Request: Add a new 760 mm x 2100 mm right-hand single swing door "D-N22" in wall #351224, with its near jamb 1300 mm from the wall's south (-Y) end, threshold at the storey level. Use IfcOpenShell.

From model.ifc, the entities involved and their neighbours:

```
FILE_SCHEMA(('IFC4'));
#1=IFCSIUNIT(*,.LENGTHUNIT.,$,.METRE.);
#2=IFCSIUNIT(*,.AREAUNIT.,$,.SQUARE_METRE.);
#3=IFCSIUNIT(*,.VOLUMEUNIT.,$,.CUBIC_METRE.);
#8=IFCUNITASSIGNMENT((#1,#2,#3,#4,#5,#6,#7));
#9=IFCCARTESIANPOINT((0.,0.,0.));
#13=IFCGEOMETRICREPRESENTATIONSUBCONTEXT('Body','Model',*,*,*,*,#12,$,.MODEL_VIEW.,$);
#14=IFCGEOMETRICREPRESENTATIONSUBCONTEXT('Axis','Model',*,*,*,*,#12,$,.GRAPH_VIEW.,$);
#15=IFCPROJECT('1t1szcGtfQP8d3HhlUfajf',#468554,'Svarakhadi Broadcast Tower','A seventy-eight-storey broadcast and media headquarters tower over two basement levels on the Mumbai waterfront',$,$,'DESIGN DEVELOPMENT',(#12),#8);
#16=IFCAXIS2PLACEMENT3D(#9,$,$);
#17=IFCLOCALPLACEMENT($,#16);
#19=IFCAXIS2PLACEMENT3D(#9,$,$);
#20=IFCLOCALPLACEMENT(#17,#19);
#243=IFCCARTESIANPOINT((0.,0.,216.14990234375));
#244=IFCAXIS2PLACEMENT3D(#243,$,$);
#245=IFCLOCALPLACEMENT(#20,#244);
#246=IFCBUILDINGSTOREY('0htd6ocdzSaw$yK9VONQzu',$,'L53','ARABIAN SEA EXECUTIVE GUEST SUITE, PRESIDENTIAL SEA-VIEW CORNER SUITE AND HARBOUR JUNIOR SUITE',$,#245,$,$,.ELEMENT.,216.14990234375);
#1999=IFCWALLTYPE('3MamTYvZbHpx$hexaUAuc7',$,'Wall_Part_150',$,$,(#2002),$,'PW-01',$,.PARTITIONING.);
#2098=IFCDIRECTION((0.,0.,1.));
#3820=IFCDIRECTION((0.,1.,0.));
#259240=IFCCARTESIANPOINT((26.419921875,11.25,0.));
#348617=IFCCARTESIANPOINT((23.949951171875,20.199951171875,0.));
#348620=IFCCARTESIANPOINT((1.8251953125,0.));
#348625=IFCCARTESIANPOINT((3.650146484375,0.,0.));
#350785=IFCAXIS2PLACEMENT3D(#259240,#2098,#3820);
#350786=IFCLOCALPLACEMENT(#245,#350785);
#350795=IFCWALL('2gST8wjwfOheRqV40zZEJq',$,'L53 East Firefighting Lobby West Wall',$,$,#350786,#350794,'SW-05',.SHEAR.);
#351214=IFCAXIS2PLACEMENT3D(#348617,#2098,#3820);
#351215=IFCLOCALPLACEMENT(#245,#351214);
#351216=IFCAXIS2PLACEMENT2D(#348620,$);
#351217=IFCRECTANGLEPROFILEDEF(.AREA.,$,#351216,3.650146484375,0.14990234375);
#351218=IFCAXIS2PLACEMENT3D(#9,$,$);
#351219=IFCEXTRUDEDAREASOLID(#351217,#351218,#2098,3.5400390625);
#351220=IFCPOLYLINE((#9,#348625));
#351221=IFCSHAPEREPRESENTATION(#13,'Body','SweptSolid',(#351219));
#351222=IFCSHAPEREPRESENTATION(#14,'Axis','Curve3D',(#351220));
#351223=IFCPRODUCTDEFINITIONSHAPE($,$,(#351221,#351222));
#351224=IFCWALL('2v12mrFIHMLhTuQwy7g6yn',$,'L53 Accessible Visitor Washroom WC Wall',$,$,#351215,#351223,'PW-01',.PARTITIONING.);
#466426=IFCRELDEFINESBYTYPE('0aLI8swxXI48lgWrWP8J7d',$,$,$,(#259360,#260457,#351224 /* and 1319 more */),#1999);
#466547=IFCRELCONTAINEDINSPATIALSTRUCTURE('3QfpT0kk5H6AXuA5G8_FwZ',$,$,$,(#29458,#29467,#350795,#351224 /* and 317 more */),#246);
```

```python
import numpy as np
import ifcopenshell
import ifcopenshell.api.feature
import ifcopenshell.api.geometry
import ifcopenshell.api.root
import ifcopenshell.api.spatial
import ifcopenshell.geom
import ifcopenshell.util.element
import ifcopenshell.util.placement
import ifcopenshell.util.representation
import ifcopenshell.util.shape
import ifcopenshell.util.unit

model = ifcopenshell.open("model.ifc")
unit_scale = ifcopenshell.util.unit.calculate_unit_scale(model)
settings = ifcopenshell.geom.settings()


def volume(element):
    """Net volume in cubic metres, openings subtracted."""
    shape = ifcopenshell.geom.create_shape(settings, element)
    return ifcopenshell.util.shape.get_volume(shape.geometry)


wall = model.by_id(351224)
storey = ifcopenshell.util.element.get_container(wall, ifc_class="IfcBuildingStorey")
context = ifcopenshell.util.representation.get_context(model, "Model", "Body", "MODEL_VIEW")
before = volume(wall)

width, height, from_end, sill = 0.76, 2.1, 1.3, 0.0  # metres

# The wall runs along its own X axis, and the end named is its -X end.
wall_shape = ifcopenshell.geom.create_shape(settings, wall)
x, y, z = ifcopenshell.util.shape.get_vertices(wall_shape.geometry).T
start = x.min() + from_end
face, thickness = float(y.min()), float(y.max() - y.min())
wall_matrix = ifcopenshell.util.placement.get_local_placement(wall.ObjectPlacement)
level = ifcopenshell.util.placement.get_local_placement(storey.ObjectPlacement)[2, 3]


def in_wall(x, y):
    """Placement at x, y metres in the wall's axes, at sill height."""
    matrix = wall_matrix.copy()
    matrix[:, 3] = wall_matrix @ np.array([x / unit_scale, y / unit_scale, 0.0, 1.0])
    matrix[2, 3] = level + sill / unit_scale
    return matrix


# Opening: a box that overshoots both wall faces by 50 mm.
opening = ifcopenshell.api.root.create_entity(model, ifc_class="IfcOpeningElement", predefined_type="OPENING")
box = ifcopenshell.api.geometry.add_wall_representation(
    model, context=context, length=width, height=height, thickness=thickness + 0.1
)
ifcopenshell.api.geometry.assign_representation(model, product=opening, representation=box)
ifcopenshell.api.geometry.edit_object_placement(model, product=opening, matrix=in_wall(start, face - 0.05), is_si=False)
ifcopenshell.api.feature.add_feature(model, feature=opening, element=wall)

door = ifcopenshell.api.root.create_entity(model, ifc_class="IfcDoor", name="D-N22", predefined_type="DOOR")
door.OverallWidth, door.OverallHeight = width / unit_scale, height / unit_scale
door.OperationType = "SINGLE_SWING_RIGHT"
body = ifcopenshell.api.geometry.add_door_representation(
    model,
    context=context,
    overall_width=door.OverallWidth,
    overall_height=door.OverallHeight,
    operation_type="SINGLE_SWING_RIGHT",
    lining_properties={"LiningDepth": thickness / unit_scale, "ThresholdDepth": thickness / unit_scale},
)
ifcopenshell.api.geometry.assign_representation(model, product=door, representation=body)
ifcopenshell.api.spatial.assign_container(model, products=[door], relating_structure=storey)
ifcopenshell.api.feature.add_filling(model, opening=opening, element=door)

# The lining spans the wall, so the door starts at the wall face.
ifcopenshell.api.geometry.edit_object_placement(model, product=door, matrix=in_wall(start, face), is_si=False)

after = volume(wall)

print(f"wall volume {before:.3f} -> {after:.3f} m3")

model.write("model-out.ifc")
```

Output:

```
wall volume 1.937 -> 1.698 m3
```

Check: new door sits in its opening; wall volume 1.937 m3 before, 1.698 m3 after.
